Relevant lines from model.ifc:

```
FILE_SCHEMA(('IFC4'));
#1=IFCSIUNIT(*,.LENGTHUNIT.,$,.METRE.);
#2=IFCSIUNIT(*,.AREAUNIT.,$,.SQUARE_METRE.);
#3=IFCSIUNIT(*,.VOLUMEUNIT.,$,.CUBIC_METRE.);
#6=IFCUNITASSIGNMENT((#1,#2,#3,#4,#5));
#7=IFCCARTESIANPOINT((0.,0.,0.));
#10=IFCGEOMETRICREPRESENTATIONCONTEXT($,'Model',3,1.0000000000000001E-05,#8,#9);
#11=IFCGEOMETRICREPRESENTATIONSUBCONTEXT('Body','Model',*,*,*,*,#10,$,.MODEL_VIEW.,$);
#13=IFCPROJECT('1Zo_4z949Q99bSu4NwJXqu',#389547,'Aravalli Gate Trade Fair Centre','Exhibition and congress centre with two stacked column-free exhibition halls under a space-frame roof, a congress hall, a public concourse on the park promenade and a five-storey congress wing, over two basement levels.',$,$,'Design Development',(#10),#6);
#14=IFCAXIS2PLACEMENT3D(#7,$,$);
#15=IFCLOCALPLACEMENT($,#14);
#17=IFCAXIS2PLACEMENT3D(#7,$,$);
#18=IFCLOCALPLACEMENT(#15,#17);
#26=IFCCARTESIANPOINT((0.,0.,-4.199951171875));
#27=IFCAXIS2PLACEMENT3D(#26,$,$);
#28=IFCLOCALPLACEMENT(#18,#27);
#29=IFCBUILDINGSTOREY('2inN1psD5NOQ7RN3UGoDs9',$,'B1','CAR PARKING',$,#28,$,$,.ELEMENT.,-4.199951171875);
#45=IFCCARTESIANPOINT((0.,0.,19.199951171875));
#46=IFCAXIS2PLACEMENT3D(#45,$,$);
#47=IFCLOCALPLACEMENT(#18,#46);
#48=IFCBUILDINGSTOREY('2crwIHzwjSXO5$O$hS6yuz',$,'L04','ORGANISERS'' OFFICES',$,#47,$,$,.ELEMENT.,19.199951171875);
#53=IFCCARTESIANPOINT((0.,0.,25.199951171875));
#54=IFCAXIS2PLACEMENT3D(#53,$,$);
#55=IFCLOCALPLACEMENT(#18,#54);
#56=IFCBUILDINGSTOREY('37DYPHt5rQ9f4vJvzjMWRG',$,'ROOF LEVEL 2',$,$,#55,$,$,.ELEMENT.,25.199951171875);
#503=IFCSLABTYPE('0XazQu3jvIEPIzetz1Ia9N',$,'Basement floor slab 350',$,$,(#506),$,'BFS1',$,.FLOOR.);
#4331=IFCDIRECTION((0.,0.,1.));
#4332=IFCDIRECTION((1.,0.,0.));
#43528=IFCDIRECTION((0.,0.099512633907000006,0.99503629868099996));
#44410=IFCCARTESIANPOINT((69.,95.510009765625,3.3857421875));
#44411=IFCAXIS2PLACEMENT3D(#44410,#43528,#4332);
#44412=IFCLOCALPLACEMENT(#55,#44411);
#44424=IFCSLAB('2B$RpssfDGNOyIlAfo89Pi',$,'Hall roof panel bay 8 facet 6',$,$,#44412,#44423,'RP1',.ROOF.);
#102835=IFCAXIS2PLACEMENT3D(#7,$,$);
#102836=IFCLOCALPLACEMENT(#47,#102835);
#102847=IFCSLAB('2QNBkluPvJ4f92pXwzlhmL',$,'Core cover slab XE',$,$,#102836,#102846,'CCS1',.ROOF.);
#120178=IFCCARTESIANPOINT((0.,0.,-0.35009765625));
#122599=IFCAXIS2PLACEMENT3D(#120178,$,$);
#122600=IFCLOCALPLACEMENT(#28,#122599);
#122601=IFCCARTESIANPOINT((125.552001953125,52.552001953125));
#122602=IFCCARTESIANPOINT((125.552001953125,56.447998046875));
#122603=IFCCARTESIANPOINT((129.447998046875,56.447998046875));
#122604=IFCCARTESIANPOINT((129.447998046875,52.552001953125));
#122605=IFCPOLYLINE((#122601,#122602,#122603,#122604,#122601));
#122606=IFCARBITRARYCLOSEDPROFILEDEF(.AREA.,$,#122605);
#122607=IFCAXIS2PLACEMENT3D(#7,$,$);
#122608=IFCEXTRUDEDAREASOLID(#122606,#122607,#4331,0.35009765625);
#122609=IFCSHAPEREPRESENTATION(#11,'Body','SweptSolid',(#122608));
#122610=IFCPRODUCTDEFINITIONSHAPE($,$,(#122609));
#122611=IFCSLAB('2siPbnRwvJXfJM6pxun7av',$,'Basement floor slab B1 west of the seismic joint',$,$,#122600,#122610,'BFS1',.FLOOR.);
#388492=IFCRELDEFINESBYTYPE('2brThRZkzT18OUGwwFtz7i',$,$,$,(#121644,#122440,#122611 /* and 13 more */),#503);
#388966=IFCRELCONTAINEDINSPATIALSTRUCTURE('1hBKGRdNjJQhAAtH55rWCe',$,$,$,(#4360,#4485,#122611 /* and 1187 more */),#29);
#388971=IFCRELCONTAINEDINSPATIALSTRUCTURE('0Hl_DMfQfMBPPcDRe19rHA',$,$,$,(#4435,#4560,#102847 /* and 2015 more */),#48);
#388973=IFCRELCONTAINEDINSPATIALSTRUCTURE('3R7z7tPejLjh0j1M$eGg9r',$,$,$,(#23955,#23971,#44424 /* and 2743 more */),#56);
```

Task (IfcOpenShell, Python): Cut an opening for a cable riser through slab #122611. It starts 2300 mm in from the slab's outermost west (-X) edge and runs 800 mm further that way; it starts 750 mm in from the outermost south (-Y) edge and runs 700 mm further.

```python
import numpy as np
import ifcopenshell
import ifcopenshell.api.feature
import ifcopenshell.api.geometry
import ifcopenshell.api.root
import ifcopenshell.geom
import ifcopenshell.util.placement
import ifcopenshell.util.representation
import ifcopenshell.util.shape
import ifcopenshell.util.unit

model = ifcopenshell.open("model.ifc")
unit_scale = ifcopenshell.util.unit.calculate_unit_scale(model)
settings = ifcopenshell.geom.settings()


def volume(element):
    """Net volume in cubic metres, openings subtracted."""
    shape = ifcopenshell.geom.create_shape(settings, element)
    return ifcopenshell.util.shape.get_volume(shape.geometry)


slab = model.by_guid("2siPbnRwvJXfJM6pxun7av")
before = volume(slab)

# Extent in the slab's own axes, in metres. The edges named are its -X and -Y sides.
slab_shape = ifcopenshell.geom.create_shape(settings, slab)
vertices = ifcopenshell.util.shape.get_vertices(slab_shape.geometry)
x_min, y_min, bottom = vertices.min(axis=0)
top = vertices[:, 2].max()

opening = ifcopenshell.api.root.create_entity(model, ifc_class="IfcOpeningElement", name="Cable riser opening", predefined_type="OPENING")
context = ifcopenshell.util.representation.get_context(model, "Model", "Body", "MODEL_VIEW")
width, depth = 0.8, 0.7
outline = [(0.0, 0.0), (width, 0.0), (width, depth), (0.0, depth), (0.0, 0.0)]
# Overshoot both faces by 50 mm so the cut is clean.
shape = ifcopenshell.api.geometry.add_slab_representation(
    model, context=context, depth=top - bottom + 0.1, polyline=outline
)
ifcopenshell.api.geometry.assign_representation(model, product=opening, representation=shape)

matrix = ifcopenshell.util.placement.get_local_placement(slab.ObjectPlacement)
matrix[:, 3] = matrix @ np.append(np.array([x_min + 2.3, y_min + 0.75, bottom - 0.05]) / unit_scale, 1.0)
ifcopenshell.api.geometry.edit_object_placement(model, product=opening, matrix=matrix, is_si=False)
ifcopenshell.api.feature.add_feature(model, feature=opening, element=slab)

after = volume(slab)

print(f"slab volume {before:.3f} -> {after:.3f} m3")

model.write("model-out.ifc")
```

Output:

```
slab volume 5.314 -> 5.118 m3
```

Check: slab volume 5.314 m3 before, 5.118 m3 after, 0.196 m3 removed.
